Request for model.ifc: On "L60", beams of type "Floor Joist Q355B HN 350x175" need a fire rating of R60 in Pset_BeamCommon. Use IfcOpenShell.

First a look at what the model holds.

```python
import ifcopenshell
import ifcopenshell.util.element

model = ifcopenshell.open("model.ifc")
print(model.schema)
storey = next(s for s in model.by_type("IfcBuildingStorey") if s.Name == "L60")
beams = [e for e in ifcopenshell.util.element.get_decomposition(storey) if e.is_a("IfcBeam")]
seen = {}
for e in beams:
    element_type = ifcopenshell.util.element.get_type(e)
    key = (element_type.Name if element_type != e and element_type else None, ifcopenshell.util.element.get_pset(e, "Pset_BeamCommon", "FireRating"))
    seen[key] = seen.get(key, 0) + 1
for (name, value), count in sorted(seen.items(), key=str):
    print(count, "x", name, "|", value)
```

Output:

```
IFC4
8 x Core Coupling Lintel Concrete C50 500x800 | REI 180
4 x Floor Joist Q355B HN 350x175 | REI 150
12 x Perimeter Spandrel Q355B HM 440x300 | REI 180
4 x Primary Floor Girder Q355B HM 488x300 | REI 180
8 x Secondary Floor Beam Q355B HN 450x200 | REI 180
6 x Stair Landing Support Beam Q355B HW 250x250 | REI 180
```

```python
import ifcopenshell
import ifcopenshell.api.pset
import ifcopenshell.util.element

model = ifcopenshell.open("model.ifc")

storey = next(s for s in model.by_type("IfcBuildingStorey") if s.Name == "L60")
beams = [e for e in ifcopenshell.util.element.get_decomposition(storey) if e.is_a("IfcBeam")]

count = 0
for e in beams:
    element_type = ifcopenshell.util.element.get_type(e)
    if element_type in (None, e) or element_type.Name != "Floor Joist Q355B HN 350x175":
        continue
    found = ifcopenshell.util.element.get_pset(e, "Pset_BeamCommon", should_inherit=False)
    if found:
        pset = model.by_id(found["id"])
        if len(ifcopenshell.util.element.get_elements_by_pset(pset)) > 1:
            pset = ifcopenshell.api.pset.unshare_pset(model, products=[e], pset=pset)[0]
    else:
        pset = ifcopenshell.api.pset.add_pset(model, product=e, name="Pset_BeamCommon")
    ifcopenshell.api.pset.edit_pset(model, pset=pset, properties={"FireRating": "R60"})
    count += 1

print(count, "beams updated")

model.write("model_v2.ifc")
```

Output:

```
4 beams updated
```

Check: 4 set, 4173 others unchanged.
